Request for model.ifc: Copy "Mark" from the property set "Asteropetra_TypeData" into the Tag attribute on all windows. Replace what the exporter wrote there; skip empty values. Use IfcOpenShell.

First a look at what the model holds.

```python
import ifcopenshell
import ifcopenshell.util.element

model = ifcopenshell.open("model.ifc")
print(model.schema)
windows = model.by_type("IfcWindow")
print(len(windows), "windows")
for e in windows[:8]:
    source = ifcopenshell.util.element.get_pset(e, "Asteropetra_TypeData", "Mark")
    target = e.Tag
    print(e.id(), repr(source), repr(target), sep=" | ")
```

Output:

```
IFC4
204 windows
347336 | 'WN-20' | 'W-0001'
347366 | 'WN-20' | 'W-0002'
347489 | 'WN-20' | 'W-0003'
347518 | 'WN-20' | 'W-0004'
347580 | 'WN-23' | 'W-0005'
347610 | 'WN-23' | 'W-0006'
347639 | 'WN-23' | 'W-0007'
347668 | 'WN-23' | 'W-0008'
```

```python
import ifcopenshell
import ifcopenshell.util.element

model = ifcopenshell.open("model.ifc")

count = 0
for e in model.by_type("IfcWindow"):
    value = ifcopenshell.util.element.get_pset(e, "Asteropetra_TypeData", "Mark")
    current = e.Tag
    if not value or not value.strip() or current == value:
        continue
    e.Tag = value
    count += 1

print(count, "windows updated")

model.write("model_updated.ifc")
```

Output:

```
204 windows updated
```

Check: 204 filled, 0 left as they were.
